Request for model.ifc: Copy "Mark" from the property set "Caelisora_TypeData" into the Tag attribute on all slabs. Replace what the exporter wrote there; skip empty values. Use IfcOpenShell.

First a look at what the model holds.

```python
import ifcopenshell
import ifcopenshell.util.element

model = ifcopenshell.open("model.ifc")
print(model.schema)
slabs = model.by_type("IfcSlab")
print(len(slabs), "slabs")
for e in slabs[:8]:
    source = ifcopenshell.util.element.get_pset(e, "Caelisora_TypeData", "Mark")
    target = e.Tag
    print(e.id(), repr(source), repr(target), sep=" | ")
```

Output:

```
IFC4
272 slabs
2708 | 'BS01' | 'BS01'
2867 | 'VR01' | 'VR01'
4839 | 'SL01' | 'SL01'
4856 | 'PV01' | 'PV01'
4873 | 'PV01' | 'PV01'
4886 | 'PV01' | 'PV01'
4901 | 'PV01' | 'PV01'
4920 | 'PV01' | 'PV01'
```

```python
import ifcopenshell
import ifcopenshell.util.element

model = ifcopenshell.open("model.ifc")

count = 0
for e in model.by_type("IfcSlab"):
    value = ifcopenshell.util.element.get_pset(e, "Caelisora_TypeData", "Mark")
    current = e.Tag
    if not value or not value.strip() or current == value:
        continue
    e.Tag = value
    count += 1

print(count, "slabs updated")

model.write("model_edited.ifc")
```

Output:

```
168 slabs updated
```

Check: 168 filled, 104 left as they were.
